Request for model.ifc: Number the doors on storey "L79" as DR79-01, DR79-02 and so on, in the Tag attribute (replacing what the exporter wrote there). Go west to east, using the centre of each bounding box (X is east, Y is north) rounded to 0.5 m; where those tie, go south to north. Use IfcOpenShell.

First a look at what the model holds.

```python
import ifcopenshell
import ifcopenshell.util.element
import ifcopenshell.util.placement

model = ifcopenshell.open("model.ifc")
print(model.schema)
storey = next(s for s in model.by_type("IfcBuildingStorey") if s.Name == "L79")
doors = [e for e in ifcopenshell.util.element.get_decomposition(storey) if e.is_a("IfcDoor")]
for e in sorted(doors, key=lambda e: e.id()):
    origin = ifcopenshell.util.placement.get_local_placement(e.ObjectPlacement)[:3, 3]
    print(e.id(), e.Tag, e.Name, origin.round(2) + 0.0, sep=" | ")
```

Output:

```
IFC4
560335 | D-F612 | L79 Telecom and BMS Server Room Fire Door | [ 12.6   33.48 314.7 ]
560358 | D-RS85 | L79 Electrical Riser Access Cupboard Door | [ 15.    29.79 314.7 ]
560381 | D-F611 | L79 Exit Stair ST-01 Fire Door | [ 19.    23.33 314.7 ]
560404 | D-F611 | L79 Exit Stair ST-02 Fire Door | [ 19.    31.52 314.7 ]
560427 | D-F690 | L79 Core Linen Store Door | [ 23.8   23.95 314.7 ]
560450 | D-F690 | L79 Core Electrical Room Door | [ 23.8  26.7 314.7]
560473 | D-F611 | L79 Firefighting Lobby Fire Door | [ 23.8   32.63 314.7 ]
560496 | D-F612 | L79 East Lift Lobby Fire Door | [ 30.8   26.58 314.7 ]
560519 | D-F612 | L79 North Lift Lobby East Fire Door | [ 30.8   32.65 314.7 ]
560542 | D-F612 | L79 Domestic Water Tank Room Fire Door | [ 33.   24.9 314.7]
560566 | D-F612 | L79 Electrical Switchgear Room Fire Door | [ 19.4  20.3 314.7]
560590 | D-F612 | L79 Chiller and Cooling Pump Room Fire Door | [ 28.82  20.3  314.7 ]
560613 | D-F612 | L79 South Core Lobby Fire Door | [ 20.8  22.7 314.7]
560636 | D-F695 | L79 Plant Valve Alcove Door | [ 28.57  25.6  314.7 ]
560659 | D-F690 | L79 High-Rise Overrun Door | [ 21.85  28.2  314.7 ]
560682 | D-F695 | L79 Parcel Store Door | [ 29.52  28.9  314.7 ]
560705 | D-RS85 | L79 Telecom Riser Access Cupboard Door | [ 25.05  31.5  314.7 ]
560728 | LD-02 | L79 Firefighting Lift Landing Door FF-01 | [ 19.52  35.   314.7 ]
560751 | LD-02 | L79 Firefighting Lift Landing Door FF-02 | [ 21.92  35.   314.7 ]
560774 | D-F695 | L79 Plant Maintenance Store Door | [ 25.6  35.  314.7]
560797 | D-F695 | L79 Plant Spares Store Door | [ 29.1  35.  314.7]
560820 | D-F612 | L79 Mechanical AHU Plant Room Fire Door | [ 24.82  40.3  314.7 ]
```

```python
import ifcopenshell
import ifcopenshell.geom
import ifcopenshell.util.element
import ifcopenshell.util.shape

model = ifcopenshell.open("model.ifc")
settings = ifcopenshell.geom.settings()
settings.set("use-world-coords", True)


def centre(element):
    shape = ifcopenshell.geom.create_shape(settings, element)
    return ifcopenshell.util.shape.get_bbox_centroid(shape.geometry)


storey = next(s for s in model.by_type("IfcBuildingStorey") if s.Name == "L79")
doors = [e for e in ifcopenshell.util.element.get_decomposition(storey) if e.is_a("IfcDoor")]

# Insertion points can sit at a corner or the storey origin, so sort by the geometry (in metres).
centres = {e: centre(e) for e in doors}
doors.sort(key=lambda e: (round(centres[e][0] / 0.5), centres[e][1]))

for i, e in enumerate(doors, start=1):
    number = f"DR79-{i:02d}"
    e.Tag = number
    print(e.id(), number)

model.write("model_rev.ifc")
```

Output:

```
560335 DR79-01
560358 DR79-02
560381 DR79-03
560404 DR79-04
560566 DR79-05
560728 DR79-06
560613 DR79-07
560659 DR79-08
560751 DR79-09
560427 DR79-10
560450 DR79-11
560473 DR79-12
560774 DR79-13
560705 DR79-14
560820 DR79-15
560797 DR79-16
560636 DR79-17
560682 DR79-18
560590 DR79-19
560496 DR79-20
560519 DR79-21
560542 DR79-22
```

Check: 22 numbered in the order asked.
